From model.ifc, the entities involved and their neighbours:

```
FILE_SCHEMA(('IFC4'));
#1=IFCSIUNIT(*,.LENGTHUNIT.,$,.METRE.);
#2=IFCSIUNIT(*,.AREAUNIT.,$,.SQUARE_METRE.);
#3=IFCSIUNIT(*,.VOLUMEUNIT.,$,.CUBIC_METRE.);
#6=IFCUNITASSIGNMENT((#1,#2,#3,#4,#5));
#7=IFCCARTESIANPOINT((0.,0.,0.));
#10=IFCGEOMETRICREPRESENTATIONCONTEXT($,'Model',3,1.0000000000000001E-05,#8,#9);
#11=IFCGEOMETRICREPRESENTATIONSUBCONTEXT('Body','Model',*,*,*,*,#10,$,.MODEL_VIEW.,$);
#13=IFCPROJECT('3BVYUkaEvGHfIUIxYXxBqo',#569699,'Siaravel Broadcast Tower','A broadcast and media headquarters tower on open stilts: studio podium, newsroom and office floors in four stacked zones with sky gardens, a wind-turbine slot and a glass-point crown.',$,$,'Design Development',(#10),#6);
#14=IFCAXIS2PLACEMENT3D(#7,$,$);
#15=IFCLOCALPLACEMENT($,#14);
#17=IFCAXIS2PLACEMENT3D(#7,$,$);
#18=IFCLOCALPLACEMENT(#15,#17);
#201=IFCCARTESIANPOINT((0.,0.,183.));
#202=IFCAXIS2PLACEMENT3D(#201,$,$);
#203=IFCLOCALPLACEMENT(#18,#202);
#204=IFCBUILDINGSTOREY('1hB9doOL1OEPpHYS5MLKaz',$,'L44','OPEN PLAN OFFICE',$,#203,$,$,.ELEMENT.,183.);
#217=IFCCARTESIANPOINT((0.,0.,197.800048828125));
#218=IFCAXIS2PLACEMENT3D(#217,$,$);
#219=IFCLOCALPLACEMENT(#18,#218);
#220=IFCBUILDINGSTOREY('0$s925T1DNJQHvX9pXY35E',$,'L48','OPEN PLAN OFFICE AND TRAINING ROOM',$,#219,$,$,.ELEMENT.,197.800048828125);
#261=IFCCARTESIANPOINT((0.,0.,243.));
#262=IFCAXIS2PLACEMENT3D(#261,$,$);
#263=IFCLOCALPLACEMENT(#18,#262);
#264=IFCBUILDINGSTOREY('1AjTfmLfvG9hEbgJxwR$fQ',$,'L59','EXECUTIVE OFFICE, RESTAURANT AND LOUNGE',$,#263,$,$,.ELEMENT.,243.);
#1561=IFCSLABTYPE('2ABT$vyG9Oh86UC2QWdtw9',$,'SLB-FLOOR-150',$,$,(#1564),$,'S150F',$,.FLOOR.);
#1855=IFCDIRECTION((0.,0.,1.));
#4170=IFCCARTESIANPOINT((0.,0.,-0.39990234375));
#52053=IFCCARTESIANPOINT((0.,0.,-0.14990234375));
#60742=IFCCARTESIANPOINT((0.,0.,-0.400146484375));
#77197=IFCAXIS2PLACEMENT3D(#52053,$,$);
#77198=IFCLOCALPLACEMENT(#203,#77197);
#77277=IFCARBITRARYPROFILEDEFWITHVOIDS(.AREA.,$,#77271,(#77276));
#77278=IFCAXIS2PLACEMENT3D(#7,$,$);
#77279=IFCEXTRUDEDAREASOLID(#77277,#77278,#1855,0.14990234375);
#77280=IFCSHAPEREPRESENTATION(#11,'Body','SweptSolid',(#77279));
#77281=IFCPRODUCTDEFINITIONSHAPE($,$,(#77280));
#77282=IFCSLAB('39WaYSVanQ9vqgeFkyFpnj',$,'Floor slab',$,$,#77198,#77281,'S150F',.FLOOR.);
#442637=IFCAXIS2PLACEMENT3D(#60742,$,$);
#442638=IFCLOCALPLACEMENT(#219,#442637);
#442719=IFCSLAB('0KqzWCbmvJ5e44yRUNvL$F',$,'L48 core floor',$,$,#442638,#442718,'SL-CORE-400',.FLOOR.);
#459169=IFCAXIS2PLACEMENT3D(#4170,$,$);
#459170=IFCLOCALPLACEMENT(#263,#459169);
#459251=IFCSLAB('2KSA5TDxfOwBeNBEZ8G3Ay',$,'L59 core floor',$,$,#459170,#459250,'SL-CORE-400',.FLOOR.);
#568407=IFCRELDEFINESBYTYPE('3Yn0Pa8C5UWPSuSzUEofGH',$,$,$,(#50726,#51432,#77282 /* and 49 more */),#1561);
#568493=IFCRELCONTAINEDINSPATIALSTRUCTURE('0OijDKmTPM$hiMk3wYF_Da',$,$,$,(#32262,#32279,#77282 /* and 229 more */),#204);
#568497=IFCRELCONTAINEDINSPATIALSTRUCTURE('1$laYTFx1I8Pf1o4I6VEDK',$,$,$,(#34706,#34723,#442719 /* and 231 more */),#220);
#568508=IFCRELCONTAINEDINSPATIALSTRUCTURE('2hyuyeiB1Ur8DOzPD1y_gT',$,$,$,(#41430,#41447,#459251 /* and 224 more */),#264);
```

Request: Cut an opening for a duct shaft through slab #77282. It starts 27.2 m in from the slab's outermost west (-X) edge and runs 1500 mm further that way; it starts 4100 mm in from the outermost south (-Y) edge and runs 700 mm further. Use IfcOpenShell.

```python
import numpy as np
import ifcopenshell
import ifcopenshell.api.feature
import ifcopenshell.api.geometry
import ifcopenshell.api.root
import ifcopenshell.geom
import ifcopenshell.util.placement
import ifcopenshell.util.representation
import ifcopenshell.util.shape
import ifcopenshell.util.unit

model = ifcopenshell.open("model.ifc")
unit_scale = ifcopenshell.util.unit.calculate_unit_scale(model)
settings = ifcopenshell.geom.settings()


def volume(element):
    """Net volume in cubic metres, openings subtracted."""
    shape = ifcopenshell.geom.create_shape(settings, element)
    return ifcopenshell.util.shape.get_volume(shape.geometry)


slab = model.by_id(77282)
before = volume(slab)

# Extent in the slab's own axes, in metres. The edges named are its -X and -Y sides.
slab_shape = ifcopenshell.geom.create_shape(settings, slab)
vertices = ifcopenshell.util.shape.get_vertices(slab_shape.geometry)
x_min, y_min, bottom = vertices.min(axis=0)
top = vertices[:, 2].max()

opening = ifcopenshell.api.root.create_entity(model, ifc_class="IfcOpeningElement", name="Duct shaft opening", predefined_type="OPENING")
context = ifcopenshell.util.representation.get_context(model, "Model", "Body", "MODEL_VIEW")
width, depth = 1.5, 0.7
outline = [(0.0, 0.0), (width, 0.0), (width, depth), (0.0, depth), (0.0, 0.0)]
# Overshoot both faces by 50 mm so the cut is clean.
shape = ifcopenshell.api.geometry.add_slab_representation(
    model, context=context, depth=top - bottom + 0.1, polyline=outline
)
ifcopenshell.api.geometry.assign_representation(model, product=opening, representation=shape)

matrix = ifcopenshell.util.placement.get_local_placement(slab.ObjectPlacement)
matrix[:, 3] = matrix @ np.append(np.array([x_min + 27.2, y_min + 4.1, bottom - 0.05]) / unit_scale, 1.0)
ifcopenshell.api.geometry.edit_object_placement(model, product=opening, matrix=matrix, is_si=False)
ifcopenshell.api.feature.add_feature(model, feature=opening, element=slab)

after = volume(slab)

print(f"slab volume {before:.3f} -> {after:.3f} m3")

model.write("model_rev.ifc")
```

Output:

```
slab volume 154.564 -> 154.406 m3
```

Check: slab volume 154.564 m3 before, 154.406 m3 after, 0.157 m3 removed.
